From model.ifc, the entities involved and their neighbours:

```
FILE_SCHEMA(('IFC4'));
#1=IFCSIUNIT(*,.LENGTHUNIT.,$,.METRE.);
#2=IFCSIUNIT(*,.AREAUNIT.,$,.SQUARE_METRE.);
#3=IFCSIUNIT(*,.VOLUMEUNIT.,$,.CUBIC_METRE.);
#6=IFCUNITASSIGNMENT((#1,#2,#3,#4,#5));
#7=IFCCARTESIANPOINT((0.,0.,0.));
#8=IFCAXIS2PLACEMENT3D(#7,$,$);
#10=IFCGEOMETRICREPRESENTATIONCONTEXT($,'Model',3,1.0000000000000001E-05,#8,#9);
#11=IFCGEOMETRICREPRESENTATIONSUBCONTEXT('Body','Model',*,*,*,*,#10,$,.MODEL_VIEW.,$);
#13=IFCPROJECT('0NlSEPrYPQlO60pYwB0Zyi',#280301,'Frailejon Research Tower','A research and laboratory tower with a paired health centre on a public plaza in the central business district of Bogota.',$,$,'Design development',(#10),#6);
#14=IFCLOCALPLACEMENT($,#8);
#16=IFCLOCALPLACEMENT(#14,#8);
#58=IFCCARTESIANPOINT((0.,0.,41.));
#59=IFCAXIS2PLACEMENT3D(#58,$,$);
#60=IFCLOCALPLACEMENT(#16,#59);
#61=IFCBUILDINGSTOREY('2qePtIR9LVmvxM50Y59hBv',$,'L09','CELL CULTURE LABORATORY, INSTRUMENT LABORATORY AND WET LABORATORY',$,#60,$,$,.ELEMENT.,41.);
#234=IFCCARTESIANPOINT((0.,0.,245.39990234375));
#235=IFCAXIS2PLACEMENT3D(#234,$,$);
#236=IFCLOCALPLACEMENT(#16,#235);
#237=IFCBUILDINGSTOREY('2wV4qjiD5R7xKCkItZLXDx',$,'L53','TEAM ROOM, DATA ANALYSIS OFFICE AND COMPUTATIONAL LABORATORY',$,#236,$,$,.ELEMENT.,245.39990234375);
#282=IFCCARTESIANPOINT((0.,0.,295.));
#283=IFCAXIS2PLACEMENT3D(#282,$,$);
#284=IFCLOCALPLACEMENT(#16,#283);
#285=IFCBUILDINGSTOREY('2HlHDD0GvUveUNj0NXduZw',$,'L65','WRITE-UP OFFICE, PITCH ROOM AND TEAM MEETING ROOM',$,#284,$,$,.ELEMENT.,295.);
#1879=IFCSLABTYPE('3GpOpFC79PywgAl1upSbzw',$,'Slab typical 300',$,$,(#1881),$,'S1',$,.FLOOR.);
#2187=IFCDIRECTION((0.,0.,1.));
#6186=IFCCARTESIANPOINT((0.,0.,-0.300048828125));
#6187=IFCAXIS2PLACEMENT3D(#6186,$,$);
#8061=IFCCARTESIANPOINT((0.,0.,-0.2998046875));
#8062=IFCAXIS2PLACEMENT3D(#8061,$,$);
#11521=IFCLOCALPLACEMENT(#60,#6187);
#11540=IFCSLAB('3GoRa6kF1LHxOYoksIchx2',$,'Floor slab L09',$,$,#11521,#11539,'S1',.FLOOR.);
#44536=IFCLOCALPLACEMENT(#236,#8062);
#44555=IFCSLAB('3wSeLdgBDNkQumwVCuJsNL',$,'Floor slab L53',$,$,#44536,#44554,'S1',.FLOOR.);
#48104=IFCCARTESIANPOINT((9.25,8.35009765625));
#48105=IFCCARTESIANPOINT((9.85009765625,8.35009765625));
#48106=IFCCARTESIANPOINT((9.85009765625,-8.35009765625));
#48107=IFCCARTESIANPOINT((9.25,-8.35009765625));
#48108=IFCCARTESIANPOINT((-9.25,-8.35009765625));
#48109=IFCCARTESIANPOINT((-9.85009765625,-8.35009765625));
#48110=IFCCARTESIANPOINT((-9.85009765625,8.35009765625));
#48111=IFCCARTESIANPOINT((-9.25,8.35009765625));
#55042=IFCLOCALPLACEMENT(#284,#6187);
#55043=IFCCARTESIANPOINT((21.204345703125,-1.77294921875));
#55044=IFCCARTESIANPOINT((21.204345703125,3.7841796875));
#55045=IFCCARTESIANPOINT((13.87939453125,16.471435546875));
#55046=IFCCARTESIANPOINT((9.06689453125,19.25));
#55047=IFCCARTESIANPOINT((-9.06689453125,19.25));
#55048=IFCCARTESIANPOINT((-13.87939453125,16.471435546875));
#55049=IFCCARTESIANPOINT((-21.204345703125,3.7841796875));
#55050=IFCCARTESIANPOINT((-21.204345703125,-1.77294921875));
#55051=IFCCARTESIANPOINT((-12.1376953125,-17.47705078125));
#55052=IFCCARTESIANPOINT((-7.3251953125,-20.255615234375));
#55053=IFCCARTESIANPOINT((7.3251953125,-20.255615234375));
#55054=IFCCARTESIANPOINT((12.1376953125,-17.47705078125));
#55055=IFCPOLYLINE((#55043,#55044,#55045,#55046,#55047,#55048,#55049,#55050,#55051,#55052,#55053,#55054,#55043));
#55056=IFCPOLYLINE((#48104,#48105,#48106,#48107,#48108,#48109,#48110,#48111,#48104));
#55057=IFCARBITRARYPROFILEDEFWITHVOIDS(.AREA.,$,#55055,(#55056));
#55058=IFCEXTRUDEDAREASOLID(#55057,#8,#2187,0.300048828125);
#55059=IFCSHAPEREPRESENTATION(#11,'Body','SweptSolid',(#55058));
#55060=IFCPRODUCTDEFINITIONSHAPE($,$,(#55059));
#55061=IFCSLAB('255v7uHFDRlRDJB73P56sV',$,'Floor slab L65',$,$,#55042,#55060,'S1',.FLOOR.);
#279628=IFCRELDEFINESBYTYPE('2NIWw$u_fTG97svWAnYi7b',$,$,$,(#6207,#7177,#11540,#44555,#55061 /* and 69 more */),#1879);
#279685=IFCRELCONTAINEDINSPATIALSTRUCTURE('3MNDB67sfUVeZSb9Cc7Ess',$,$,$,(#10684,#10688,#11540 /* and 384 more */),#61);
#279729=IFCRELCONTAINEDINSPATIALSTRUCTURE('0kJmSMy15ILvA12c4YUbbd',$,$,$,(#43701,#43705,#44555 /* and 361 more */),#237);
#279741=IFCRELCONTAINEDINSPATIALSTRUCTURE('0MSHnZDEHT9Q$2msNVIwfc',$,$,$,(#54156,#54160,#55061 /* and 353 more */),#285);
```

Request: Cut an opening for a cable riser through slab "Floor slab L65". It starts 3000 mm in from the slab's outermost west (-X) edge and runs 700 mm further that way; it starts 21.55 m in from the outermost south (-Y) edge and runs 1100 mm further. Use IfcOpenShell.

```python
import numpy as np
import ifcopenshell
import ifcopenshell.api.feature
import ifcopenshell.api.geometry
import ifcopenshell.api.root
import ifcopenshell.geom
import ifcopenshell.util.placement
import ifcopenshell.util.representation
import ifcopenshell.util.shape
import ifcopenshell.util.unit

model = ifcopenshell.open("model.ifc")
unit_scale = ifcopenshell.util.unit.calculate_unit_scale(model)
settings = ifcopenshell.geom.settings()


def volume(element):
    """Net volume in cubic metres, openings subtracted."""
    shape = ifcopenshell.geom.create_shape(settings, element)
    return ifcopenshell.util.shape.get_volume(shape.geometry)


slab = model.by_id(55061)
before = volume(slab)

# Extent in the slab's own axes, in metres. The edges named are its -X and -Y sides.
slab_shape = ifcopenshell.geom.create_shape(settings, slab)
vertices = ifcopenshell.util.shape.get_vertices(slab_shape.geometry)
x_min, y_min, bottom = vertices.min(axis=0)
top = vertices[:, 2].max()

opening = ifcopenshell.api.root.create_entity(model, ifc_class="IfcOpeningElement", name="Cable riser opening", predefined_type="OPENING")
context = ifcopenshell.util.representation.get_context(model, "Model", "Body", "MODEL_VIEW")
width, depth = 0.7, 1.1
outline = [(0.0, 0.0), (width, 0.0), (width, depth), (0.0, depth), (0.0, 0.0)]
# Overshoot both faces by 50 mm so the cut is clean.
shape = ifcopenshell.api.geometry.add_slab_representation(
    model, context=context, depth=top - bottom + 0.1, polyline=outline
)
ifcopenshell.api.geometry.assign_representation(model, product=opening, representation=shape)

matrix = ifcopenshell.util.placement.get_local_placement(slab.ObjectPlacement)
matrix[:, 3] = matrix @ np.append(np.array([x_min + 3, y_min + 21.55, bottom - 0.05]) / unit_scale, 1.0)
ifcopenshell.api.geometry.edit_object_placement(model, product=opening, matrix=matrix, is_si=False)
ifcopenshell.api.feature.add_feature(model, feature=opening, element=slab)

after = volume(slab)

print(f"slab volume {before:.3f} -> {after:.3f} m3")

model.write("model_updated.ifc")
```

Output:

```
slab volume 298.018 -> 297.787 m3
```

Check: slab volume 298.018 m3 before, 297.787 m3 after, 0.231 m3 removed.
